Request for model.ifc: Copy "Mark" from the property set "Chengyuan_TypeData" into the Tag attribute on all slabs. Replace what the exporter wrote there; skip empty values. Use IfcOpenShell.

First a look at what the model holds.

```python
import ifcopenshell
import ifcopenshell.util.element

model = ifcopenshell.open("model.ifc")
print(model.schema)
slabs = model.by_type("IfcSlab")
print(len(slabs), "slabs")
for e in slabs[:8]:
    source = ifcopenshell.util.element.get_pset(e, "Chengyuan_TypeData", "Mark")
    target = e.Tag
    print(e.id(), repr(source), repr(target), sep=" | ")
```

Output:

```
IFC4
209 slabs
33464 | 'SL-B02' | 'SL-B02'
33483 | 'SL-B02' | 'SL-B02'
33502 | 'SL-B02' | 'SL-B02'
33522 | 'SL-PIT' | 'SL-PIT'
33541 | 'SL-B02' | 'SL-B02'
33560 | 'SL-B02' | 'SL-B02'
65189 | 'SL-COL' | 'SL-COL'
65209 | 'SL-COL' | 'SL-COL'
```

```python
import ifcopenshell
import ifcopenshell.util.element

model = ifcopenshell.open("model.ifc")

count = 0
for e in model.by_type("IfcSlab"):
    value = ifcopenshell.util.element.get_pset(e, "Chengyuan_TypeData", "Mark")
    current = e.Tag
    if not value or not value.strip() or current == value:
        continue
    e.Tag = value
    count += 1

print(count, "slabs updated")

model.write("model-out.ifc")
```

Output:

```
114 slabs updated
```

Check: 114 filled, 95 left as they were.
